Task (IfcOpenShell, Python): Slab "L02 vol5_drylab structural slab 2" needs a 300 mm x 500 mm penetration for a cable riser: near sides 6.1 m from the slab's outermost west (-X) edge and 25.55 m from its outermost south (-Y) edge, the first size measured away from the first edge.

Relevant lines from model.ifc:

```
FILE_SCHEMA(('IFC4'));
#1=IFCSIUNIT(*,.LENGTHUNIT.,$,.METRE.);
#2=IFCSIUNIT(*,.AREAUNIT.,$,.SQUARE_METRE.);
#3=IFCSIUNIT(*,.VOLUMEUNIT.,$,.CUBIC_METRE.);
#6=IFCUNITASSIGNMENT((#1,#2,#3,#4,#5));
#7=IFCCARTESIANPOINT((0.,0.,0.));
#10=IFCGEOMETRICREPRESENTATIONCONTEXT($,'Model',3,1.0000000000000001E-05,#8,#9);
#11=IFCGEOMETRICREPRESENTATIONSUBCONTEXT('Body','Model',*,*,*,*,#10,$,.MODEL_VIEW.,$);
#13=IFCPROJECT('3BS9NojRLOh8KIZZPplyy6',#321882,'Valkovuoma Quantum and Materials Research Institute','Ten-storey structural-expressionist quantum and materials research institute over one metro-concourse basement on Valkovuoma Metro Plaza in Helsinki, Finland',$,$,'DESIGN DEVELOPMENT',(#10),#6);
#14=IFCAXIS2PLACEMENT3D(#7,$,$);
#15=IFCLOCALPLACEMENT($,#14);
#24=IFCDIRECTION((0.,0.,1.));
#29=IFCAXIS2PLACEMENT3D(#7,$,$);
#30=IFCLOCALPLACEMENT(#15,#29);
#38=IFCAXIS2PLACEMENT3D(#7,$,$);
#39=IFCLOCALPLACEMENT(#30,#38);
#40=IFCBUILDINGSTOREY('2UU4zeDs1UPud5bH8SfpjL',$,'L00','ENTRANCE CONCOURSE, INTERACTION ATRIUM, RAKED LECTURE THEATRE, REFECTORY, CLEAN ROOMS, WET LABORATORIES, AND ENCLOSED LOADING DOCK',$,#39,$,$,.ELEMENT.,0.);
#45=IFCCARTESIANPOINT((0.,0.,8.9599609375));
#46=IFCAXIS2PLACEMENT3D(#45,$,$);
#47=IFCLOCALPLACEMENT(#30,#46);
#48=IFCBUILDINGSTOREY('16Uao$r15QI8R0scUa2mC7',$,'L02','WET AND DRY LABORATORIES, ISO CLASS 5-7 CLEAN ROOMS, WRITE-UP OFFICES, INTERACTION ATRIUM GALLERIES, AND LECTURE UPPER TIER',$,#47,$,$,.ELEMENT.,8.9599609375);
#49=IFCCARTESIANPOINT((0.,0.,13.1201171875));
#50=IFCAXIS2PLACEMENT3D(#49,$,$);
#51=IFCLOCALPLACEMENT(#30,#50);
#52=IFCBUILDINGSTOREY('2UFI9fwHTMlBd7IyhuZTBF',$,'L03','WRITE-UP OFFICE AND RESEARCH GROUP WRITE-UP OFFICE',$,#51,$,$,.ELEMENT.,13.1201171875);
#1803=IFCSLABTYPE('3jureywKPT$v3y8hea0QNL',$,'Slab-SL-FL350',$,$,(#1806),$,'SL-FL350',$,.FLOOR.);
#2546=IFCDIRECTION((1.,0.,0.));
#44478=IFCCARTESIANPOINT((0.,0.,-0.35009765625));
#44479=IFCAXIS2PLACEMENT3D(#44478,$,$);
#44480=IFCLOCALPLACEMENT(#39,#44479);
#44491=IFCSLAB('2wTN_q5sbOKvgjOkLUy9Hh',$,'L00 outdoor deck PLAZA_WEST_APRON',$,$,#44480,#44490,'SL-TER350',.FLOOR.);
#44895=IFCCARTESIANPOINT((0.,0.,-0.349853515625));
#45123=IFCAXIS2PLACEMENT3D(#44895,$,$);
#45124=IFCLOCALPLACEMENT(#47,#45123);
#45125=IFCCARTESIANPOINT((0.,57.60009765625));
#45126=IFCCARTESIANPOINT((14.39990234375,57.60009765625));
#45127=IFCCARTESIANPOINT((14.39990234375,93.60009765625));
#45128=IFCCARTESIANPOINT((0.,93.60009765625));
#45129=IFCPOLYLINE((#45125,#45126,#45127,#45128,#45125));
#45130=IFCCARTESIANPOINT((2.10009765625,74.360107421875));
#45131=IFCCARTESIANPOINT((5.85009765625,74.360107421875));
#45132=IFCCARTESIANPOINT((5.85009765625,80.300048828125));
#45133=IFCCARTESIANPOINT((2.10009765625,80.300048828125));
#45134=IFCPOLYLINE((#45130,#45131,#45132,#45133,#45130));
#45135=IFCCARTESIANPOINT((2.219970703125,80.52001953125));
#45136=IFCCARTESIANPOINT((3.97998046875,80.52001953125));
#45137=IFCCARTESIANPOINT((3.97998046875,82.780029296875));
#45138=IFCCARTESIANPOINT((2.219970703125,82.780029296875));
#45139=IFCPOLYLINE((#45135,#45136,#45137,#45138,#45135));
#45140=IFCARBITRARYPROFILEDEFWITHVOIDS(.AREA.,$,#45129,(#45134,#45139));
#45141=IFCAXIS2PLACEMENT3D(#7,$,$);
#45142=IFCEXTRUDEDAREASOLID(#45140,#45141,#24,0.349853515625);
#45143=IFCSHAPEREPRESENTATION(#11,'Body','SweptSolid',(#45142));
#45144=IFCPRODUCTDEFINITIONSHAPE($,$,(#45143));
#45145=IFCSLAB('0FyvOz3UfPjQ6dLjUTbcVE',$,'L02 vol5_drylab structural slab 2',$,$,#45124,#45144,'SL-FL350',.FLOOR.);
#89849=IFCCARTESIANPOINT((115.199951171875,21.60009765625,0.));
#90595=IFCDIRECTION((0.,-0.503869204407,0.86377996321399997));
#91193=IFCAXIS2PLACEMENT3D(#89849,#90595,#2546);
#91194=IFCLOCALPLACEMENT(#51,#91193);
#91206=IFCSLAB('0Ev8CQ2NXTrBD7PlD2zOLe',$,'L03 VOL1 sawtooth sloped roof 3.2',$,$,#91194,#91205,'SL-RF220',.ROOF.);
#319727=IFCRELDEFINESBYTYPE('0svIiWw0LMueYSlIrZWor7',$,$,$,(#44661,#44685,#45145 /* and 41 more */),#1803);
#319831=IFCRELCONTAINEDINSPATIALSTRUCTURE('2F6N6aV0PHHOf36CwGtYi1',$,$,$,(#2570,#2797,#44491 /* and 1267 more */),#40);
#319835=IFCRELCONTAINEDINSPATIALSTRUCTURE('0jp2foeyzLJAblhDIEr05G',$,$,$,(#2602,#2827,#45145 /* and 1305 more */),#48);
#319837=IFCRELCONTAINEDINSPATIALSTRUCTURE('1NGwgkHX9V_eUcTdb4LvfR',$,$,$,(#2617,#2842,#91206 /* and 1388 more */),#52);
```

```python
import numpy as np
import ifcopenshell
import ifcopenshell.api.feature
import ifcopenshell.api.geometry
import ifcopenshell.api.root
import ifcopenshell.geom
import ifcopenshell.util.placement
import ifcopenshell.util.representation
import ifcopenshell.util.shape
import ifcopenshell.util.unit

model = ifcopenshell.open("model.ifc")
unit_scale = ifcopenshell.util.unit.calculate_unit_scale(model)
settings = ifcopenshell.geom.settings()


def volume(element):
    """Net volume in cubic metres, openings subtracted."""
    shape = ifcopenshell.geom.create_shape(settings, element)
    return ifcopenshell.util.shape.get_volume(shape.geometry)


slab = model.by_guid("0FyvOz3UfPjQ6dLjUTbcVE")
before = volume(slab)

# Extent in the slab's own axes, in metres. The edges named are its -X and -Y sides.
slab_shape = ifcopenshell.geom.create_shape(settings, slab)
vertices = ifcopenshell.util.shape.get_vertices(slab_shape.geometry)
x_min, y_min, bottom = vertices.min(axis=0)
top = vertices[:, 2].max()

opening = ifcopenshell.api.root.create_entity(model, ifc_class="IfcOpeningElement", name="Cable riser opening", predefined_type="OPENING")
context = ifcopenshell.util.representation.get_context(model, "Model", "Body", "MODEL_VIEW")
width, depth = 0.3, 0.5
outline = [(0.0, 0.0), (width, 0.0), (width, depth), (0.0, depth), (0.0, 0.0)]
# Overshoot both faces by 50 mm so the cut is clean.
shape = ifcopenshell.api.geometry.add_slab_representation(
    model, context=context, depth=top - bottom + 0.1, polyline=outline
)
ifcopenshell.api.geometry.assign_representation(model, product=opening, representation=shape)

matrix = ifcopenshell.util.placement.get_local_placement(slab.ObjectPlacement)
matrix[:, 3] = matrix @ np.append(np.array([x_min + 6.1, y_min + 25.55, bottom - 0.05]) / unit_scale, 1.0)
ifcopenshell.api.geometry.edit_object_placement(model, product=opening, matrix=matrix, is_si=False)
ifcopenshell.api.feature.add_feature(model, feature=opening, element=slab)

after = volume(slab)

print(f"slab volume {before:.3f} -> {after:.3f} m3")

model.write("model_updated.ifc")
```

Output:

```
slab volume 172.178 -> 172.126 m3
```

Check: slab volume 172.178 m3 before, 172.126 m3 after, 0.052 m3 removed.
